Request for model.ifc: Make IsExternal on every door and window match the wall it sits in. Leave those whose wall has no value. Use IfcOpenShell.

First a look at what the model holds.

```python
import ifcopenshell
import ifcopenshell.util.element

model = ifcopenshell.open("model.ifc")
print(model.schema)
seen = {}
for e in model.by_type("IfcDoor") + model.by_type("IfcWindow"):
    if not e.FillsVoids:
        continue
    host = e.FillsVoids[0].RelatingOpeningElement.VoidsElements[0].RelatingBuildingElement
    own = ifcopenshell.util.element.get_pset(e, f"Pset_{e.is_a()[3:].removesuffix('StandardCase')}Common", "IsExternal")
    wall = ifcopenshell.util.element.get_pset(host, "Pset_WallCommon", "IsExternal")
    seen[e.is_a(), own, wall] = seen.get((e.is_a(), own, wall), 0) + 1
for (cls, own, wall), count in sorted(seen.items(), key=str):
    print(count, cls, "IsExternal:", own, "| host wall:", wall)
```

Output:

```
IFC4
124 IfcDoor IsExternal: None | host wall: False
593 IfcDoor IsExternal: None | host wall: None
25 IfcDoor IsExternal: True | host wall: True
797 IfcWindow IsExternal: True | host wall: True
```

```python
import ifcopenshell
import ifcopenshell.api.pset
import ifcopenshell.util.element

model = ifcopenshell.open("model.ifc")

count = 0
for ifc_class, pset_name in (("IfcDoor", "Pset_DoorCommon"), ("IfcWindow", "Pset_WindowCommon")):
    for e in model.by_type(ifc_class):
        if not e.FillsVoids:
            continue
        host = e.FillsVoids[0].RelatingOpeningElement.VoidsElements[0].RelatingBuildingElement
        external = ifcopenshell.util.element.get_pset(host, "Pset_WallCommon", "IsExternal")
        if external is None or ifcopenshell.util.element.get_pset(e, pset_name, "IsExternal") == external:
            continue
        pset = ifcopenshell.api.pset.add_pset(model, product=e, name=pset_name)
        ifcopenshell.api.pset.edit_pset(model, pset=pset, properties={"IsExternal": external})
        count += 1

print(count, "updated")

model.write("model-out.ifc")
```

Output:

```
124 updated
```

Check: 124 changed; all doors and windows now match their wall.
